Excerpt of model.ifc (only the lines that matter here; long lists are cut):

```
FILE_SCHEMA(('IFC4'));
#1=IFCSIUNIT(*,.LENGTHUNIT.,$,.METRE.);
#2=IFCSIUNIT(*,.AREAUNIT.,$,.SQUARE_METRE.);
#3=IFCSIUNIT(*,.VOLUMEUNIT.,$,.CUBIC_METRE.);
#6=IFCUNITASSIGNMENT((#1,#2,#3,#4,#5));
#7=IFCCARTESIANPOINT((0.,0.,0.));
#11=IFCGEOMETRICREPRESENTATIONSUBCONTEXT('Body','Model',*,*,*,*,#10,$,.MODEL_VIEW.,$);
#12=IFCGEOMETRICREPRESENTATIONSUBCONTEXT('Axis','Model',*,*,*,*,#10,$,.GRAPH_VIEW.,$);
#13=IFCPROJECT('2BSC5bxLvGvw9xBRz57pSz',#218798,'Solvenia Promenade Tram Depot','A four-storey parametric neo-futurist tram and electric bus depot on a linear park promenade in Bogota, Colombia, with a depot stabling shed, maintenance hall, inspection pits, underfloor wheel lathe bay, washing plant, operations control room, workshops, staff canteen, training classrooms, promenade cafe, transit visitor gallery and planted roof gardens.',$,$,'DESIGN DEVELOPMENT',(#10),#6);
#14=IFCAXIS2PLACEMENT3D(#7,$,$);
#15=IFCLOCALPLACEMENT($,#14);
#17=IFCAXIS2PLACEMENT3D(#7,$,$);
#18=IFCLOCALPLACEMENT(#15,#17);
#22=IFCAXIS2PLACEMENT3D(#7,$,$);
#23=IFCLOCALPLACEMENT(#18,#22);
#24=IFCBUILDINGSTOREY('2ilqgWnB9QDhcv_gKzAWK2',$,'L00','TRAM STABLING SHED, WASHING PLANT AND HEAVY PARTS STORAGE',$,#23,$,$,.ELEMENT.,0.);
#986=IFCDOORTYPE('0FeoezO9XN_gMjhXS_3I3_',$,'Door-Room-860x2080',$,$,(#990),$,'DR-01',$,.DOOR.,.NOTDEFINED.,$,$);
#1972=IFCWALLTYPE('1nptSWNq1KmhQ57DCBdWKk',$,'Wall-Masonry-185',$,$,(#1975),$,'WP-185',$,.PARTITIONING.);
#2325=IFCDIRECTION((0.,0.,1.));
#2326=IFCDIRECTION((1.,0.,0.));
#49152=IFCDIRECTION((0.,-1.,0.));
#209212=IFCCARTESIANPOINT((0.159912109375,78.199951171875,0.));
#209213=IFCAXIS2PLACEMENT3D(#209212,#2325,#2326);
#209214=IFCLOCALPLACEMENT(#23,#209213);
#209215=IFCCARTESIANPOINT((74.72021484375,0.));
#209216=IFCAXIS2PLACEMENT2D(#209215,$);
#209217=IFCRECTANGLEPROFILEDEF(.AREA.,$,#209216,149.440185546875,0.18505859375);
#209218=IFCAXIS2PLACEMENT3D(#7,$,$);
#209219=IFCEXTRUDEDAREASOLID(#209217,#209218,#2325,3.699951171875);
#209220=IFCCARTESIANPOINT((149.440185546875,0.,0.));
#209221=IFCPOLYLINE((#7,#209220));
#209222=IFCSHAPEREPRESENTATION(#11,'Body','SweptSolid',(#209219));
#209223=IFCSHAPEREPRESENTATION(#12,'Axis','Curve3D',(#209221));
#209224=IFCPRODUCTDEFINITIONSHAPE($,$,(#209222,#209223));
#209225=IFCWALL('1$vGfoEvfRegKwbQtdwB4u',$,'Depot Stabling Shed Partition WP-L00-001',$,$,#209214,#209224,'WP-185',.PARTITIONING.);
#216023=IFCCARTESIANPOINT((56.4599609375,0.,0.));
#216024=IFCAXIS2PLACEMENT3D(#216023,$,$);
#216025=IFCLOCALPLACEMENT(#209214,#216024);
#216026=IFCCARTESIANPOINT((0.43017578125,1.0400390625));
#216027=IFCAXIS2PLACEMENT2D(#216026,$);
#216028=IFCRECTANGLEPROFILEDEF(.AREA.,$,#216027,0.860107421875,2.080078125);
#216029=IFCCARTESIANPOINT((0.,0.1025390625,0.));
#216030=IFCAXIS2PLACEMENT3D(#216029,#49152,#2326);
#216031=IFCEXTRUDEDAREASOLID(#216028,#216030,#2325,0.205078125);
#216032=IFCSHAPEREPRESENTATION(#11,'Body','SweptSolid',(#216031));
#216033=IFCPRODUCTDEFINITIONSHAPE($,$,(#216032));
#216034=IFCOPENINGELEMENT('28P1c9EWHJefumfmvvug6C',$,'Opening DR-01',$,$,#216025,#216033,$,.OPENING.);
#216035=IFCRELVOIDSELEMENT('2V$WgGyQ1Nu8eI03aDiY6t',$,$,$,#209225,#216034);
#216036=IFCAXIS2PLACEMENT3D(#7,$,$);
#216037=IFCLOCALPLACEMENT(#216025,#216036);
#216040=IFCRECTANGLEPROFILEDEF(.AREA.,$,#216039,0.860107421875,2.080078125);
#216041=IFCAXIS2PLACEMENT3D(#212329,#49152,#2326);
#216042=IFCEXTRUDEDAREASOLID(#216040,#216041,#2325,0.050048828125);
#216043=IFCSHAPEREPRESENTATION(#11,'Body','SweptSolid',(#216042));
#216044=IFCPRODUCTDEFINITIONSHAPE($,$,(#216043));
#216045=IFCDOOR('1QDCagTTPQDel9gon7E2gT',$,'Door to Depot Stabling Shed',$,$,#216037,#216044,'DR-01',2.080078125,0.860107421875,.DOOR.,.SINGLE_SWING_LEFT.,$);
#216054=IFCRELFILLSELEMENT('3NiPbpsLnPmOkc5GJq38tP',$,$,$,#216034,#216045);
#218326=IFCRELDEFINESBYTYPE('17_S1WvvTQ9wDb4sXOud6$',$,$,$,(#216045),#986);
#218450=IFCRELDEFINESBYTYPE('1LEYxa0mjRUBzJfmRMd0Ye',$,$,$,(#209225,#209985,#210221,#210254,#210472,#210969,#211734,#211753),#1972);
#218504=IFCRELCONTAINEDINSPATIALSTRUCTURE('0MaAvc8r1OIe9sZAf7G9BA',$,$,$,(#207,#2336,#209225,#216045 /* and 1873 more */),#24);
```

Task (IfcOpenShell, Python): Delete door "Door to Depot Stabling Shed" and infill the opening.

```python
import ifcopenshell
import ifcopenshell.api.feature
import ifcopenshell.api.root
import ifcopenshell.geom
import ifcopenshell.util.shape

model = ifcopenshell.open("model.ifc")
settings = ifcopenshell.geom.settings()


def volume(element):
    """Net volume in cubic metres, openings subtracted."""
    shape = ifcopenshell.geom.create_shape(settings, element)
    return ifcopenshell.util.shape.get_volume(shape.geometry)


door = model.by_guid("1QDCagTTPQDel9gon7E2gT")
opening = door.FillsVoids[0].RelatingOpeningElement
wall = opening.VoidsElements[0].RelatingBuildingElement
before = volume(wall)

ifcopenshell.api.root.remove_product(model, product=door)
ifcopenshell.api.feature.remove_feature(model, feature=opening)

after = volume(wall)

print(f"wall volume {before:.3f} -> {after:.3f} m3")

model.write("model_v2.ifc")
```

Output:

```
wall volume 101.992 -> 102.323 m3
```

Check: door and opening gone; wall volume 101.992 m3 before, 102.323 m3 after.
